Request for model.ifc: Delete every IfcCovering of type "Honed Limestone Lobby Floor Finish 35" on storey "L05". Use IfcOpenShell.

First a look at what the model holds.

```python
import ifcopenshell
import ifcopenshell.util.element

model = ifcopenshell.open("model.ifc")
print(model.schema)
storey = next(s for s in model.by_type("IfcBuildingStorey") if s.Name == "L05")
coverings = [e for e in ifcopenshell.util.element.get_decomposition(storey) if e.is_a("IfcCovering")]
seen = {}
for e in coverings:
    element_type = ifcopenshell.util.element.get_type(e)
    name = element_type.Name if element_type not in (None, e) else None
    seen[name] = seen.get(name, 0) + 1
for name, count in sorted(seen.items(), key=str):
    print(count, "x", name)
```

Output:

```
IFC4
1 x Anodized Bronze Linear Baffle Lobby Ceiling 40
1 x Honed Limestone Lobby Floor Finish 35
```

```python
import ifcopenshell
import ifcopenshell.api.root
import ifcopenshell.util.element

model = ifcopenshell.open("model.ifc")

storey = next(s for s in model.by_type("IfcBuildingStorey") if s.Name == "L05")
coverings = [e for e in ifcopenshell.util.element.get_decomposition(storey) if e.is_a("IfcCovering")]
targets = [e for e in coverings if (t := ifcopenshell.util.element.get_type(e)) not in (None, e) and t.Name == "Honed Limestone Lobby Floor Finish 35"]

for e in targets:
    ifcopenshell.api.root.remove_product(model, product=e)
print(len(targets), "removed")

model.write("model_rev.ifc")
```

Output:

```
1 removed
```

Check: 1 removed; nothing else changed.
